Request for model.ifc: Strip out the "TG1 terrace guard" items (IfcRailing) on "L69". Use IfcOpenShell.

First a look at what the model holds.

```python
import ifcopenshell
import ifcopenshell.util.element

model = ifcopenshell.open("model.ifc")
print(model.schema)
storey = next(s for s in model.by_type("IfcBuildingStorey") if s.Name == "L69")
railings = [e for e in ifcopenshell.util.element.get_decomposition(storey) if e.is_a("IfcRailing")]
seen = {}
for e in railings:
    element_type = ifcopenshell.util.element.get_type(e)
    name = element_type.Name if element_type not in (None, e) else None
    seen[name] = seen.get(name, 0) + 1
for name, count in sorted(seen.items(), key=str):
    print(count, "x", name)
```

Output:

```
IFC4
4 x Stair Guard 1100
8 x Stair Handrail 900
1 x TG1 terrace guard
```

```python
import ifcopenshell
import ifcopenshell.api.root
import ifcopenshell.util.element

model = ifcopenshell.open("model.ifc")

storey = next(s for s in model.by_type("IfcBuildingStorey") if s.Name == "L69")
railings = [e for e in ifcopenshell.util.element.get_decomposition(storey) if e.is_a("IfcRailing")]
targets = [e for e in railings if (t := ifcopenshell.util.element.get_type(e)) not in (None, e) and t.Name == "TG1 terrace guard"]

for e in targets:
    ifcopenshell.api.root.remove_product(model, product=e)
print(len(targets), "removed")

model.write("model_v2.ifc")
```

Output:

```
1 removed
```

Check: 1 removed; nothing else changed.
